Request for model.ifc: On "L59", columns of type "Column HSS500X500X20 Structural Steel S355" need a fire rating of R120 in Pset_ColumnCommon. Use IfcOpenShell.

First a look at what the model holds.

```python
import ifcopenshell
import ifcopenshell.util.element

model = ifcopenshell.open("model.ifc")
print(model.schema)
storey = next(s for s in model.by_type("IfcBuildingStorey") if s.Name == "L59")
columns = [e for e in ifcopenshell.util.element.get_decomposition(storey) if e.is_a("IfcColumn")]
seen = {}
for e in columns:
    element_type = ifcopenshell.util.element.get_type(e)
    key = (element_type.Name if element_type != e and element_type else None, ifcopenshell.util.element.get_pset(e, "Pset_ColumnCommon", "FireRating"))
    seen[key] = seen.get(key, 0) + 1
for (name, value), count in sorted(seen.items(), key=str):
    print(count, "x", name, "|", value)
```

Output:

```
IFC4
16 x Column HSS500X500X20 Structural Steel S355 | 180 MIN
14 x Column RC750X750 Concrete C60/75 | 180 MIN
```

```python
import ifcopenshell
import ifcopenshell.api.pset
import ifcopenshell.util.element

model = ifcopenshell.open("model.ifc")

storey = next(s for s in model.by_type("IfcBuildingStorey") if s.Name == "L59")
columns = [e for e in ifcopenshell.util.element.get_decomposition(storey) if e.is_a("IfcColumn")]

count = 0
for e in columns:
    element_type = ifcopenshell.util.element.get_type(e)
    if element_type in (None, e) or element_type.Name != "Column HSS500X500X20 Structural Steel S355":
        continue
    # add_pset returns the element's existing set when there is one.
    pset = ifcopenshell.api.pset.add_pset(model, product=e, name="Pset_ColumnCommon")
    ifcopenshell.api.pset.edit_pset(model, pset=pset, properties={"FireRating": "R120"})
    count += 1

print(count, "columns updated")

model.write("model-out.ifc")
```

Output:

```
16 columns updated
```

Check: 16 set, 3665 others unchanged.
